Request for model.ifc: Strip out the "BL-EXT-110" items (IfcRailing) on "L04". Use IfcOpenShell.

First a look at what the model holds.

```python
import ifcopenshell
import ifcopenshell.util.element

model = ifcopenshell.open("model.ifc")
print(model.schema)
storey = next(s for s in model.by_type("IfcBuildingStorey") if s.Name == "L04")
railings = [e for e in ifcopenshell.util.element.get_decomposition(storey) if e.is_a("IfcRailing")]
seen = {}
for e in railings:
    element_type = ifcopenshell.util.element.get_type(e)
    name = element_type.Name if element_type not in (None, e) else None
    seen[name] = seen.get(name, 0) + 1
for name, count in sorted(seen.items(), key=str):
    print(count, "x", name)
```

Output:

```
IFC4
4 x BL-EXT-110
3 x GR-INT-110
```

```python
import ifcopenshell
import ifcopenshell.api.root
import ifcopenshell.util.element

model = ifcopenshell.open("model.ifc")

storey = next(s for s in model.by_type("IfcBuildingStorey") if s.Name == "L04")
railings = [e for e in ifcopenshell.util.element.get_decomposition(storey) if e.is_a("IfcRailing")]
targets = [e for e in railings if (t := ifcopenshell.util.element.get_type(e)) not in (None, e) and t.Name == "BL-EXT-110"]

for e in targets:
    ifcopenshell.api.root.remove_product(model, product=e)
print(len(targets), "removed")

model.write("model_v2.ifc")
```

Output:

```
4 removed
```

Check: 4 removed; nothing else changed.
